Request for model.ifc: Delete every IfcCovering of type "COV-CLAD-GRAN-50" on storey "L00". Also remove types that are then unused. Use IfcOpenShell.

First a look at what the model holds.

```python
import ifcopenshell
import ifcopenshell.util.element

model = ifcopenshell.open("model.ifc")
print(model.schema)
storey = next(s for s in model.by_type("IfcBuildingStorey") if s.Name == "L00")
coverings = [e for e in ifcopenshell.util.element.get_decomposition(storey) if e.is_a("IfcCovering")]
seen = {}
for e in coverings:
    element_type = ifcopenshell.util.element.get_type(e)
    name = element_type.Name if element_type not in (None, e) else None
    seen[name] = seen.get(name, 0) + 1
for name, count in sorted(seen.items(), key=str):
    print(count, "x", name)
```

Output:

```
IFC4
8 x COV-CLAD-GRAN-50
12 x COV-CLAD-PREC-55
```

```python
import ifcopenshell
import ifcopenshell.api.root
import ifcopenshell.util.element

model = ifcopenshell.open("model.ifc")

storey = next(s for s in model.by_type("IfcBuildingStorey") if s.Name == "L00")
coverings = [e for e in ifcopenshell.util.element.get_decomposition(storey) if e.is_a("IfcCovering")]
targets = [e for e in coverings if (t := ifcopenshell.util.element.get_type(e)) not in (None, e) and t.Name == "COV-CLAD-GRAN-50"]
types = {ifcopenshell.util.element.get_type(e) for e in targets} - {None, *targets}

for e in targets:
    ifcopenshell.api.root.remove_product(model, product=e)
print(len(targets), "removed")

unused = [t for t in types if not ifcopenshell.util.element.get_types(t)]
for t in unused:
    ifcopenshell.api.root.remove_product(model, product=t)
print(len(unused), "unused types removed")

model.write("model_rev.ifc")
```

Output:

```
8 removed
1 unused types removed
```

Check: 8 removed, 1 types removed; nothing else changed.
